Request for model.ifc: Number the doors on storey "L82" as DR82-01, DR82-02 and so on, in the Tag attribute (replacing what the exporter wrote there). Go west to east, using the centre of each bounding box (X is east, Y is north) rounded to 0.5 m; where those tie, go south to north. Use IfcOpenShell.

First a look at what the model holds.

```python
import ifcopenshell
import ifcopenshell.util.element
import ifcopenshell.util.placement

model = ifcopenshell.open("model.ifc")
print(model.schema)
storey = next(s for s in model.by_type("IfcBuildingStorey") if s.Name == "L82")
doors = [e for e in ifcopenshell.util.element.get_decomposition(storey) if e.is_a("IfcDoor")]
for e in sorted(doors, key=lambda e: e.id()):
    origin = ifcopenshell.util.placement.get_local_placement(e.ObjectPlacement)[:3, 3]
    print(e.id(), e.Tag, e.Name, origin.round(2) + 0.0, sep=" | ")
```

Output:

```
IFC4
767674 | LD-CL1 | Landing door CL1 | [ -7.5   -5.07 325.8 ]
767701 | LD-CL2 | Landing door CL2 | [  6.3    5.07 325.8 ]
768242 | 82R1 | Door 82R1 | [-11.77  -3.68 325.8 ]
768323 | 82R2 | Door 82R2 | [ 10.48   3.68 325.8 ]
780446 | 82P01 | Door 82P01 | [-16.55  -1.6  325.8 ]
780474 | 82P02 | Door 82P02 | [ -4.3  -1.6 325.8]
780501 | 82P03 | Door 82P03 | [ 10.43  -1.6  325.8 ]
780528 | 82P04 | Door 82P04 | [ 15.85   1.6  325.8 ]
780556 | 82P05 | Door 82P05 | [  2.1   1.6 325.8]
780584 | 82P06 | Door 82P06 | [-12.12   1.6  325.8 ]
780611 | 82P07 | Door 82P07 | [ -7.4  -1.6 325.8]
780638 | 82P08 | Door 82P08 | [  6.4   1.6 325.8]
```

```python
import ifcopenshell
import ifcopenshell.geom
import ifcopenshell.util.element
import ifcopenshell.util.shape

model = ifcopenshell.open("model.ifc")
settings = ifcopenshell.geom.settings()
settings.set("use-world-coords", True)


def centre(element):
    shape = ifcopenshell.geom.create_shape(settings, element)
    return ifcopenshell.util.shape.get_bbox_centroid(shape.geometry)


storey = next(s for s in model.by_type("IfcBuildingStorey") if s.Name == "L82")
doors = [e for e in ifcopenshell.util.element.get_decomposition(storey) if e.is_a("IfcDoor")]

# Insertion points can sit at a corner or the storey origin, so sort by the geometry (in metres).
centres = {e: centre(e) for e in doors}
doors.sort(key=lambda e: (round(centres[e][0] / 0.5), centres[e][1]))

for i, e in enumerate(doors, start=1):
    number = f"DR82-{i:02d}"
    e.Tag = number
    print(e.id(), number)

model.write("model_updated.ifc")
```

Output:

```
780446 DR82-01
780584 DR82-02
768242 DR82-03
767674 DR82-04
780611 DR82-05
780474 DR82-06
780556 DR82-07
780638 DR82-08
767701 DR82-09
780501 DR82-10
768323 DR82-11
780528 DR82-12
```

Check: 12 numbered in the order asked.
